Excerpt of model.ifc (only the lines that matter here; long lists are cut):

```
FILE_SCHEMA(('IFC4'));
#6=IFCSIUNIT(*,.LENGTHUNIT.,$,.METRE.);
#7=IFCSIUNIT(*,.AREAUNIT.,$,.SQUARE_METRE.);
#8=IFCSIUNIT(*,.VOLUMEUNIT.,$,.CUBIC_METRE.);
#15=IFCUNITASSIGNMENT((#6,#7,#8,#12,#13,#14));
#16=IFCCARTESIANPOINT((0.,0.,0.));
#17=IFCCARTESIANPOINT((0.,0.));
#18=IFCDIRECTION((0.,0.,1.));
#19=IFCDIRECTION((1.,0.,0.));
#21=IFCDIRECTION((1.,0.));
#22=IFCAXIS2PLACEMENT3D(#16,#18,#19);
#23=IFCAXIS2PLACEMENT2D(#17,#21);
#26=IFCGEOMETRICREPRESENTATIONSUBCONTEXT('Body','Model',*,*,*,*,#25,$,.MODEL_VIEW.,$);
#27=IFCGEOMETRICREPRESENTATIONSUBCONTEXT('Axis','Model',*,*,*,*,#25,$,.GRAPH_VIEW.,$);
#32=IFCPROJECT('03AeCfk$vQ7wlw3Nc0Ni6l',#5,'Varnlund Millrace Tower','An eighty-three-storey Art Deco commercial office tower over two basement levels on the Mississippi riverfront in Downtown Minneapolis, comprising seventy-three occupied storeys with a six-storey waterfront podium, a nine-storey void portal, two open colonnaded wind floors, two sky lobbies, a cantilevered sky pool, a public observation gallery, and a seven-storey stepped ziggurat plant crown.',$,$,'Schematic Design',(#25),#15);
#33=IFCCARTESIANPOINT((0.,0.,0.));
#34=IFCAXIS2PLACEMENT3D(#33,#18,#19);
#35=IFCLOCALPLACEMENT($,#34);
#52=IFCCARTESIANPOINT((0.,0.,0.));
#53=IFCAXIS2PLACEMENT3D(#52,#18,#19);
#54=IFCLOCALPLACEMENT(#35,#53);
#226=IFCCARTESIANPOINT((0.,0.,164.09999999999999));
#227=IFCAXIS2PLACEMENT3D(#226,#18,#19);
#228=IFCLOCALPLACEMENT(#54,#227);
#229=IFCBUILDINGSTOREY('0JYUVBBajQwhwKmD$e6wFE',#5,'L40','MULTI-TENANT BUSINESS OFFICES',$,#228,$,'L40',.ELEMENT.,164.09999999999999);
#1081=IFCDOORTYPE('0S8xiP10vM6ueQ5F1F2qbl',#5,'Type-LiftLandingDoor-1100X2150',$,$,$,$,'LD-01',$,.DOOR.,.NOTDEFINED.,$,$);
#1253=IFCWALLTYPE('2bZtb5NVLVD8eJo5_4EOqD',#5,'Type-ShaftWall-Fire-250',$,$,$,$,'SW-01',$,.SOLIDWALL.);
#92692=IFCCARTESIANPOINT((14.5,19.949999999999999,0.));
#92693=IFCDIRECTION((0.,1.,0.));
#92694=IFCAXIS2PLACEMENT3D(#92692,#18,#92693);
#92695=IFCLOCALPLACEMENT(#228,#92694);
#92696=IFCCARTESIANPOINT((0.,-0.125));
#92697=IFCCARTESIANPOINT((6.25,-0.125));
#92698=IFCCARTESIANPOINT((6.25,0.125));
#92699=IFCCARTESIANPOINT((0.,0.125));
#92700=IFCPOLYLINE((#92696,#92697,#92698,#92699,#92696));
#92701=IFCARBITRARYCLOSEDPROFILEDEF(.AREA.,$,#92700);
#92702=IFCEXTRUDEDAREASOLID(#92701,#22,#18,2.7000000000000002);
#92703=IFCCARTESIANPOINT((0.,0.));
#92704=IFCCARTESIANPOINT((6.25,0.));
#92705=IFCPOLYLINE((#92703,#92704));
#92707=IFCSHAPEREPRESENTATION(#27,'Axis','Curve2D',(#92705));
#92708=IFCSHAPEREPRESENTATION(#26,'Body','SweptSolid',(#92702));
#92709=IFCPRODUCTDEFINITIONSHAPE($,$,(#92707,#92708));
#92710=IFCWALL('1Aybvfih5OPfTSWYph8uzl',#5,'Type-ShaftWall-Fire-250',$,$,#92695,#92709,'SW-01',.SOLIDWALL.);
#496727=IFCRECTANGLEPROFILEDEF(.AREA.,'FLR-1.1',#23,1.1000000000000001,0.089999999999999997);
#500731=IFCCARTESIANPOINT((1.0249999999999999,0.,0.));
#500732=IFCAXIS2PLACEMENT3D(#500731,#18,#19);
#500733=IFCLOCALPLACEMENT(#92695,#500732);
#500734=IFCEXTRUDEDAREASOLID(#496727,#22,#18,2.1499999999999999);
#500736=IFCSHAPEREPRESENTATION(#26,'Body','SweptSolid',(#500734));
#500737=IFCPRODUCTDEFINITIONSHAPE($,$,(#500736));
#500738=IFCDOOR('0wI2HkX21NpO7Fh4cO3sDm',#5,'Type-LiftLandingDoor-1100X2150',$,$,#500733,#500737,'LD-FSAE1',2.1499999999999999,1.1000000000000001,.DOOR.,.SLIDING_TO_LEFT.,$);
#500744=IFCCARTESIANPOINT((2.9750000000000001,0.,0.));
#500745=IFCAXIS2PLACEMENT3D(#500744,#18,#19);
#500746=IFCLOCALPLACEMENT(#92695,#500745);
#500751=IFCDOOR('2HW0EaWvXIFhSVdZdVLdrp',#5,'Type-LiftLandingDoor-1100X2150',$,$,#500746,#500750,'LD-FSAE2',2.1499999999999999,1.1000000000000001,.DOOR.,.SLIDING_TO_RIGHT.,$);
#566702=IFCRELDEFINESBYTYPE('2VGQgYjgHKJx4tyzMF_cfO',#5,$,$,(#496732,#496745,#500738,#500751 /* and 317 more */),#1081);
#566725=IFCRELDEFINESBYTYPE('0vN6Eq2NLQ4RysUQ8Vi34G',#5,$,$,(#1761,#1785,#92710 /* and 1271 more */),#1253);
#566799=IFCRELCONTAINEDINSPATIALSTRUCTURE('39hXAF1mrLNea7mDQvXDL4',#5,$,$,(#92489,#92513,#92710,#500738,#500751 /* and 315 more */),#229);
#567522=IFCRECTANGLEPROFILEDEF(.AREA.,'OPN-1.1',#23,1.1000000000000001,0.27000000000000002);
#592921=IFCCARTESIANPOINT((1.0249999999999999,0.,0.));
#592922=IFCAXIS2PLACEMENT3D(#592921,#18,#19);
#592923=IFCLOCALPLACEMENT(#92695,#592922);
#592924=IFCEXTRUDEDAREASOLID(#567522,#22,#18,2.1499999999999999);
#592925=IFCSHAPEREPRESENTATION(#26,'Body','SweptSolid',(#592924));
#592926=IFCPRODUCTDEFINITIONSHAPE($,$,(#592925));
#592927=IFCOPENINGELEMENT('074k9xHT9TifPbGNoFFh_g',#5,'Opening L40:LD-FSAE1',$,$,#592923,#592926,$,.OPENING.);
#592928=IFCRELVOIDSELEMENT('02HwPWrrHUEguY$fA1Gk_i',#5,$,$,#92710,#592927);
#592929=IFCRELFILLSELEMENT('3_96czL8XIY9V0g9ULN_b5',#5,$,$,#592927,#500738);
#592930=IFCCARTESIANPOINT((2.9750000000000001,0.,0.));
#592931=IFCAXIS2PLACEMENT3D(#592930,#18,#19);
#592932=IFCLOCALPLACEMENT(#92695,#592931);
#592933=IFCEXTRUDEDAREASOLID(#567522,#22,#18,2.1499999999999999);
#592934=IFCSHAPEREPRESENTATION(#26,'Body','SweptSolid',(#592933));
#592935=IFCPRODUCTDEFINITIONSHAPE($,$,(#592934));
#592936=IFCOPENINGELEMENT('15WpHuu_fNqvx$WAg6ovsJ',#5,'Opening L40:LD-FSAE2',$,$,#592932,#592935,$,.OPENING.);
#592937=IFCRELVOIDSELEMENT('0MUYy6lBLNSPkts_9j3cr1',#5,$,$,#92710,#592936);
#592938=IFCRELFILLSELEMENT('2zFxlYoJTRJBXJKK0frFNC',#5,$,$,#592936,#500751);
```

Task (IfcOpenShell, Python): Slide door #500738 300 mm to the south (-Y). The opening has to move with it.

```python
import ifcopenshell
import ifcopenshell.api.geometry
import ifcopenshell.util.placement
import ifcopenshell.util.unit

model = ifcopenshell.open("model.ifc")
unit_scale = ifcopenshell.util.unit.calculate_unit_scale(model)

door = model.by_guid("0wI2HkX21NpO7Fh4cO3sDm")
opening = door.FillsVoids[0].RelatingOpeningElement
wall = opening.VoidsElements[0].RelatingBuildingElement

wall_matrix = ifcopenshell.util.placement.get_local_placement(wall.ObjectPlacement)
shift = wall_matrix[:3, 0] * -0.3 / unit_scale
before = ifcopenshell.util.placement.get_local_placement(door.ObjectPlacement)[:3, 3].copy()

# The door is not placed relative to its opening, so move both.
for product in (opening, door):
    matrix = ifcopenshell.util.placement.get_local_placement(product.ObjectPlacement)
    matrix[:3, 3] += shift
    ifcopenshell.api.geometry.edit_object_placement(model, product=product, matrix=matrix, is_si=False)

after = ifcopenshell.util.placement.get_local_placement(door.ObjectPlacement)[:3, 3]
print("door moved by", (after - before).round(3) + 0.0)

model.write("model-out.ifc")
```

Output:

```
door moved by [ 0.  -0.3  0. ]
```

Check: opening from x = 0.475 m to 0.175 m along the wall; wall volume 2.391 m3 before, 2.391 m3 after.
